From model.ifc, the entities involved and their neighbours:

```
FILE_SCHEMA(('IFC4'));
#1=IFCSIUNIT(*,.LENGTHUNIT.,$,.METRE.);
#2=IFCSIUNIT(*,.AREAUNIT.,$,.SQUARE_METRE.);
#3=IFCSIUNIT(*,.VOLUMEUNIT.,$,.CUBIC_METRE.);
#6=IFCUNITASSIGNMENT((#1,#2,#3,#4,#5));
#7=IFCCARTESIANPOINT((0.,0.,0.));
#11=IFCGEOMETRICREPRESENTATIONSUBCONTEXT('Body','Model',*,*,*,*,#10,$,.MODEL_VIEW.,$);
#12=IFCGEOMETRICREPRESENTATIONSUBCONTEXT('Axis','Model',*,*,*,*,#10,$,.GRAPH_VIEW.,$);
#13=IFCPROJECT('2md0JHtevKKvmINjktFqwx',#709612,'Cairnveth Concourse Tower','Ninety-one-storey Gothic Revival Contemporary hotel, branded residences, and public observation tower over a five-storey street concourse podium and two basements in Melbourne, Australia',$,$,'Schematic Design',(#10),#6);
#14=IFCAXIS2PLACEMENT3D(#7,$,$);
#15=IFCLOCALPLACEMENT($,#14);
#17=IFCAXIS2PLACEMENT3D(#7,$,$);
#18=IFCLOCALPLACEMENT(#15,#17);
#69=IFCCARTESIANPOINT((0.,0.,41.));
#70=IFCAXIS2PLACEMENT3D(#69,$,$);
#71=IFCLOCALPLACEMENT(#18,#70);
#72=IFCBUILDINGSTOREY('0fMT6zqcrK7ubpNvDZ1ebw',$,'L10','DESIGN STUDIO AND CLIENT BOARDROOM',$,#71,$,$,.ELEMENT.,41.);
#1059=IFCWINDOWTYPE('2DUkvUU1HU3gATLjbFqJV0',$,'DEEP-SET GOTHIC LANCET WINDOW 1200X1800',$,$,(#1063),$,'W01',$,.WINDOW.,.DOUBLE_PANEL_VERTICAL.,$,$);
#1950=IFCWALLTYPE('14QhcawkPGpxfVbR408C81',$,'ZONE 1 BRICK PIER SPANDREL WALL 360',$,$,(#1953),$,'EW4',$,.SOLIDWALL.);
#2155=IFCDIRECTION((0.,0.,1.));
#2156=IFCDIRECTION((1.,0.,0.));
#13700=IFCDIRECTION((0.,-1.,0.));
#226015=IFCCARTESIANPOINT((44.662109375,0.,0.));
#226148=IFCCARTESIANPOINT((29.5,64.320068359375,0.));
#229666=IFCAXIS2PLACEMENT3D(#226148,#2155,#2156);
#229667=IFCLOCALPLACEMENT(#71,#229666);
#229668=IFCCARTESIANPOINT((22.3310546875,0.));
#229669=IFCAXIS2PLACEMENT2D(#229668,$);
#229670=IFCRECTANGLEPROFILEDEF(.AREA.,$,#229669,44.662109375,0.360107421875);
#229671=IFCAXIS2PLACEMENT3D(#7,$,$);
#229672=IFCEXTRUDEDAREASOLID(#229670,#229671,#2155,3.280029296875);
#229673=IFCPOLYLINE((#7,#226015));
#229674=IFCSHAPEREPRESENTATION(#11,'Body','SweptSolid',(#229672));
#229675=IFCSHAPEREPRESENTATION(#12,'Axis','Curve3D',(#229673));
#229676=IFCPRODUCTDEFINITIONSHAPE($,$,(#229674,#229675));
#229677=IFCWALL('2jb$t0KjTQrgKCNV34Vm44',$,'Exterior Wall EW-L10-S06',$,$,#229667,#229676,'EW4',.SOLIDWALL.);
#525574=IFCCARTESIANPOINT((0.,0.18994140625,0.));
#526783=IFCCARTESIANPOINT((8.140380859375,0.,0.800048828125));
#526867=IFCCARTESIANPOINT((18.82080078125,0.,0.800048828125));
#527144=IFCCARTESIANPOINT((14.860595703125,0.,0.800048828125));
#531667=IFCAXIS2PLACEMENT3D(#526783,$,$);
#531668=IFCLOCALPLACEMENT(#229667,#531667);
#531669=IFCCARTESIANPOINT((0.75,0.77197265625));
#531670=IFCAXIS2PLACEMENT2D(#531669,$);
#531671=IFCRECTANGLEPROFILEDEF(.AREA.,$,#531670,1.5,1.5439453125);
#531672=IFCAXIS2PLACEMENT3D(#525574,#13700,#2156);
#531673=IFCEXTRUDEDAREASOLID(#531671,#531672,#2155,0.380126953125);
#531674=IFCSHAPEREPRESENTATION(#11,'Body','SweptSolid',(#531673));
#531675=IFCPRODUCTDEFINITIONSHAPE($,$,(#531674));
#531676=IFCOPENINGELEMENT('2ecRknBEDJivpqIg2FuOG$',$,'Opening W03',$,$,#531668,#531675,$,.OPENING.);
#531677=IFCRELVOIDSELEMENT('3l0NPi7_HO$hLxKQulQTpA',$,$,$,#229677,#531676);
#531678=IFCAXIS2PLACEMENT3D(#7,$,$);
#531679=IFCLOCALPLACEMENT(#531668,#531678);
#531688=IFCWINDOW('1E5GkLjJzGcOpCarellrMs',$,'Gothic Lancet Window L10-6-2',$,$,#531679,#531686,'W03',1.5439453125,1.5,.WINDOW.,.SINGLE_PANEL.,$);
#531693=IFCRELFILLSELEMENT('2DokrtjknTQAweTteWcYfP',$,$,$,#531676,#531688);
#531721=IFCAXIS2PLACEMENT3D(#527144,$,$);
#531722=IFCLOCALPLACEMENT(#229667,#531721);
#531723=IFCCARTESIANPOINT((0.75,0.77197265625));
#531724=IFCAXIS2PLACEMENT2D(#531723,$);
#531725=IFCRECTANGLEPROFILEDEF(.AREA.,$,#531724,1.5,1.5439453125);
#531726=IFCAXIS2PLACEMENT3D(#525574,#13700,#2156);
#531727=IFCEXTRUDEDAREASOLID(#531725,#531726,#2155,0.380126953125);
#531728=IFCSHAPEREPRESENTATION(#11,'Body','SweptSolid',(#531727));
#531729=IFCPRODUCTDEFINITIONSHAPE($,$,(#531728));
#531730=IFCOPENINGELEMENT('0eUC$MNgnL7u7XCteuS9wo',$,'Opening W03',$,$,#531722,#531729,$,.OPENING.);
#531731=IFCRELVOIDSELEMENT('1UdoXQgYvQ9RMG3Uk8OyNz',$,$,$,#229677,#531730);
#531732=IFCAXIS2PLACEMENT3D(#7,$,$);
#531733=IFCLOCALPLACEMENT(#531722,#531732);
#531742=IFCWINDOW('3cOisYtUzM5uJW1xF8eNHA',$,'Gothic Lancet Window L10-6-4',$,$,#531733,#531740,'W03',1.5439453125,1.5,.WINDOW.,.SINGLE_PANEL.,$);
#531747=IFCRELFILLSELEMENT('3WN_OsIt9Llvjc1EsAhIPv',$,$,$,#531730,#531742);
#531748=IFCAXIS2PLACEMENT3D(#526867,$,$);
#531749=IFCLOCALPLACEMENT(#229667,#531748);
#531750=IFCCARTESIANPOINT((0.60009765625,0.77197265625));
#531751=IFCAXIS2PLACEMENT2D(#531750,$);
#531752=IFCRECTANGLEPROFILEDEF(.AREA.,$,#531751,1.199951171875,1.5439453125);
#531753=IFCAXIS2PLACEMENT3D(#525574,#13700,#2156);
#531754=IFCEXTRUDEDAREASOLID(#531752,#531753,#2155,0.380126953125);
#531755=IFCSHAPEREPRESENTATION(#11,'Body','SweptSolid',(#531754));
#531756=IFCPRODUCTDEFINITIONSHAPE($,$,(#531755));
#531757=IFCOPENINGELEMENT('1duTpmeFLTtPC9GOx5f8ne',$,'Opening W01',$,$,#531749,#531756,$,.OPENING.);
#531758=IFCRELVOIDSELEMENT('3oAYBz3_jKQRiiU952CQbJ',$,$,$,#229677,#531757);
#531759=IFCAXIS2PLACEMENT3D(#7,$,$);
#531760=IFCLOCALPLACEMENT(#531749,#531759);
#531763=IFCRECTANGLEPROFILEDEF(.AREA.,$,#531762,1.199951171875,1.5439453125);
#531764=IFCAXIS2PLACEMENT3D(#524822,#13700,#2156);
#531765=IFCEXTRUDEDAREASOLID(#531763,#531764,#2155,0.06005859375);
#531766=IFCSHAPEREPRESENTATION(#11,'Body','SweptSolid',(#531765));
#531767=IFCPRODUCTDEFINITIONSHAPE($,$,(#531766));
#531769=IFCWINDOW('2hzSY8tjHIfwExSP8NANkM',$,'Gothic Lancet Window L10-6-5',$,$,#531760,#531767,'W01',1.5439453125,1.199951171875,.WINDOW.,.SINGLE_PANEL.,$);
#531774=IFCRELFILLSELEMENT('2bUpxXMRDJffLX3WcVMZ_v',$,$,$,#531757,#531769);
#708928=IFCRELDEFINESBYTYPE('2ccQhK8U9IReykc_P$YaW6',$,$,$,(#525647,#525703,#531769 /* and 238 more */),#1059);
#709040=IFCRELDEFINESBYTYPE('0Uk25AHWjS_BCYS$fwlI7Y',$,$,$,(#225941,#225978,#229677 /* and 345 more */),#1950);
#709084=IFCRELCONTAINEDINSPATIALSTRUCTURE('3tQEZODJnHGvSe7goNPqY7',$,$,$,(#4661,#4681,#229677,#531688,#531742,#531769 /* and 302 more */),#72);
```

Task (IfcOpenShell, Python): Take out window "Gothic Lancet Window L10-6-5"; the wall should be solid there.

```python
import ifcopenshell
import ifcopenshell.api.feature
import ifcopenshell.api.root
import ifcopenshell.geom
import ifcopenshell.util.shape

model = ifcopenshell.open("model.ifc")
settings = ifcopenshell.geom.settings()


def volume(element):
    """Net volume in cubic metres, openings subtracted."""
    shape = ifcopenshell.geom.create_shape(settings, element)
    return ifcopenshell.util.shape.get_volume(shape.geometry)


window = model.by_id(531769)
opening = window.FillsVoids[0].RelatingOpeningElement
wall = opening.VoidsElements[0].RelatingBuildingElement
before = volume(wall)

ifcopenshell.api.root.remove_product(model, product=window)
ifcopenshell.api.feature.remove_feature(model, feature=opening)

after = volume(wall)

print(f"wall volume {before:.3f} -> {after:.3f} m3")

model.write("model-out.ifc")
```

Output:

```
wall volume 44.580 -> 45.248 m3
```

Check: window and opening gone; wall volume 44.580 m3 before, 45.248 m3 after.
